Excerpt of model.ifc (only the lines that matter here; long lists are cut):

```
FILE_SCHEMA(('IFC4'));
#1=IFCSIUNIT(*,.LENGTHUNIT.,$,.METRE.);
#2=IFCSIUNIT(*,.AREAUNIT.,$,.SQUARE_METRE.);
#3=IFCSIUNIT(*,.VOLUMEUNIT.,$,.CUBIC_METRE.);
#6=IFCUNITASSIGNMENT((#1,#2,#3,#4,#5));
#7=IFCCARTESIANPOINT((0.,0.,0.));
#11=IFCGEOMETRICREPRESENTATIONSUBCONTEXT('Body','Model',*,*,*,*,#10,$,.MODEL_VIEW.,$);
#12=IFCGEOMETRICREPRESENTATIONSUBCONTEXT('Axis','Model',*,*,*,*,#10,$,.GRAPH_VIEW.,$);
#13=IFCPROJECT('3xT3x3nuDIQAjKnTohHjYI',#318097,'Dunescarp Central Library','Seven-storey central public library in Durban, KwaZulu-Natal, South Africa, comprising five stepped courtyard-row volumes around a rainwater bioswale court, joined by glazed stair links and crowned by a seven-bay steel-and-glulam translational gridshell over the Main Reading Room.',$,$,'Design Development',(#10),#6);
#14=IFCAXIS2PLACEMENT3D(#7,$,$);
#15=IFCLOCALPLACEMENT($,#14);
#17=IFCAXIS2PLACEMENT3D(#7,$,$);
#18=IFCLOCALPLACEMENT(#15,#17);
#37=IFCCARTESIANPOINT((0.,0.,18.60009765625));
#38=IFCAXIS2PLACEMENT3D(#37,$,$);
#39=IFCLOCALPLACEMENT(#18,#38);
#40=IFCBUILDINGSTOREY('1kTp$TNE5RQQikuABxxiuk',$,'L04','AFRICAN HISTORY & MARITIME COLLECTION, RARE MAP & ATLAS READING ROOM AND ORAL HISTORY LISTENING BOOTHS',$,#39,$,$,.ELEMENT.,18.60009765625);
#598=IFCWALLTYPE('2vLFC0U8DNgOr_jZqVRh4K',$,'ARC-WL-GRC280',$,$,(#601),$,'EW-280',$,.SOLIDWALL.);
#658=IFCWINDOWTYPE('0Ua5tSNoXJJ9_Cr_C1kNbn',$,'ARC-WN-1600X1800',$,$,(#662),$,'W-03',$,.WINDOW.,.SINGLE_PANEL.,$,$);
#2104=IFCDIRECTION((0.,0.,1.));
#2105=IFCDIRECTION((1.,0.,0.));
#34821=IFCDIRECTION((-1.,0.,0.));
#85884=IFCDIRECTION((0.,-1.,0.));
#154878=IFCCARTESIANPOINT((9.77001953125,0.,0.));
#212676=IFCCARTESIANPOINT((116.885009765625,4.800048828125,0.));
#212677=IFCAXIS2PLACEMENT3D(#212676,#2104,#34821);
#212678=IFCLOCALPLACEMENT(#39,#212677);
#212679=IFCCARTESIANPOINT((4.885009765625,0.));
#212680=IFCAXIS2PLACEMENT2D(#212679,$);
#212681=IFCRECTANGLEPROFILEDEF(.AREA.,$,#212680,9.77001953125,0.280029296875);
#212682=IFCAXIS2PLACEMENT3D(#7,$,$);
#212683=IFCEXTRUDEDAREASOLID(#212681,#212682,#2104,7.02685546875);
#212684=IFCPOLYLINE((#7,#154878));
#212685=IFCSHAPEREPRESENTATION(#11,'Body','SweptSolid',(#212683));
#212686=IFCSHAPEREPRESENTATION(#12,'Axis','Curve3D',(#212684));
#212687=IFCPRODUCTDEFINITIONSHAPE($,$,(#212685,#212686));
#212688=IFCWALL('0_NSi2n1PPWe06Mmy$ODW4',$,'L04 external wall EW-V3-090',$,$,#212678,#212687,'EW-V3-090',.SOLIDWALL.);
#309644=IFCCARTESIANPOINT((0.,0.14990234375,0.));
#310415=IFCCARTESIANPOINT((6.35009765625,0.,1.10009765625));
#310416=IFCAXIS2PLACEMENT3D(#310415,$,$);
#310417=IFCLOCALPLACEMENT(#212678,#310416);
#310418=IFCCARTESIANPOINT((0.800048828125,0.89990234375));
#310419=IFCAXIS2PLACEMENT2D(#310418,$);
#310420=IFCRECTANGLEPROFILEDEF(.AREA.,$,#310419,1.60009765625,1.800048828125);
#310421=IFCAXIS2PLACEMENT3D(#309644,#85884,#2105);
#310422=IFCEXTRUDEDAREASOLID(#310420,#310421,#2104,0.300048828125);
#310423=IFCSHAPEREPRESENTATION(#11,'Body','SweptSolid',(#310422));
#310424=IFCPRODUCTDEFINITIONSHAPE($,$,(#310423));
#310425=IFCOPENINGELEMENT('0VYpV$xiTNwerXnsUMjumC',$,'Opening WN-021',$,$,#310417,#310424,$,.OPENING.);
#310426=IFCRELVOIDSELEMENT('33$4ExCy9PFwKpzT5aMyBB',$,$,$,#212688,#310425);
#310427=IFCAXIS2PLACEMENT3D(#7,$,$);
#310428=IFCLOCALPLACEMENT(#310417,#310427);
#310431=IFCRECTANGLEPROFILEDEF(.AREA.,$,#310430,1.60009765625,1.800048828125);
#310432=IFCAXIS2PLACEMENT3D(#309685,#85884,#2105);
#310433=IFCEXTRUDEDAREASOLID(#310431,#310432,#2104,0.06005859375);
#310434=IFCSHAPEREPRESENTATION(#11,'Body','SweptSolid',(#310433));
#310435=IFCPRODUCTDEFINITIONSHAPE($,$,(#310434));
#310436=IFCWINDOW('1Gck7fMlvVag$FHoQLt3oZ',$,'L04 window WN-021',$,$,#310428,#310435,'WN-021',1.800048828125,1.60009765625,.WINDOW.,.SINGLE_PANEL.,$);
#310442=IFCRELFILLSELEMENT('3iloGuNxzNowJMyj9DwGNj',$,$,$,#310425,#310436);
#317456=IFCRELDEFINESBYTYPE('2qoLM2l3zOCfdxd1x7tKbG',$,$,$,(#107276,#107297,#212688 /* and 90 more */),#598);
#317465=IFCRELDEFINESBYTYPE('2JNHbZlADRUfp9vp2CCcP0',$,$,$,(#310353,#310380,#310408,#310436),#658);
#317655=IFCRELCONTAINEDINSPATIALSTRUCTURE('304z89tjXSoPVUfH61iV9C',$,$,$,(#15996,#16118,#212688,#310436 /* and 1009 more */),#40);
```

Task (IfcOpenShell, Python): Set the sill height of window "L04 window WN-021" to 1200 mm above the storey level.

```python
import numpy as np
import ifcopenshell
import ifcopenshell.api.geometry
import ifcopenshell.geom
import ifcopenshell.util.element
import ifcopenshell.util.placement
import ifcopenshell.util.shape
import ifcopenshell.util.unit

model = ifcopenshell.open("model.ifc")
unit_scale = ifcopenshell.util.unit.calculate_unit_scale(model)

window = model.by_id(310436)
opening = window.FillsVoids[0].RelatingOpeningElement
storey = ifcopenshell.util.element.get_container(window, ifc_class="IfcBuildingStorey")
level = ifcopenshell.util.placement.get_local_placement(storey.ObjectPlacement)[2, 3]

# The opening's origin need not be at the sill, so measure its lowest point.
shape = ifcopenshell.geom.create_shape(ifcopenshell.geom.settings(), opening)
bottom = ifcopenshell.util.shape.get_shape_bottom_elevation(shape, shape.geometry) / unit_scale
dz = level + 1.2 / unit_scale - bottom

shift = np.array([0.0, 0.0, dz])
# The window is placed relative to its opening, so it follows when the opening moves.
matrix = ifcopenshell.util.placement.get_local_placement(opening.ObjectPlacement)
matrix[:3, 3] += shift
ifcopenshell.api.geometry.edit_object_placement(
    model, product=opening, matrix=matrix, is_si=False, should_transform_children=True
)

print(f"moved by {dz * unit_scale:+.3f} m")

model.write("model_updated.ifc")
```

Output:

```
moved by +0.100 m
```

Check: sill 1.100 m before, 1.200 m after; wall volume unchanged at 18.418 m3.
